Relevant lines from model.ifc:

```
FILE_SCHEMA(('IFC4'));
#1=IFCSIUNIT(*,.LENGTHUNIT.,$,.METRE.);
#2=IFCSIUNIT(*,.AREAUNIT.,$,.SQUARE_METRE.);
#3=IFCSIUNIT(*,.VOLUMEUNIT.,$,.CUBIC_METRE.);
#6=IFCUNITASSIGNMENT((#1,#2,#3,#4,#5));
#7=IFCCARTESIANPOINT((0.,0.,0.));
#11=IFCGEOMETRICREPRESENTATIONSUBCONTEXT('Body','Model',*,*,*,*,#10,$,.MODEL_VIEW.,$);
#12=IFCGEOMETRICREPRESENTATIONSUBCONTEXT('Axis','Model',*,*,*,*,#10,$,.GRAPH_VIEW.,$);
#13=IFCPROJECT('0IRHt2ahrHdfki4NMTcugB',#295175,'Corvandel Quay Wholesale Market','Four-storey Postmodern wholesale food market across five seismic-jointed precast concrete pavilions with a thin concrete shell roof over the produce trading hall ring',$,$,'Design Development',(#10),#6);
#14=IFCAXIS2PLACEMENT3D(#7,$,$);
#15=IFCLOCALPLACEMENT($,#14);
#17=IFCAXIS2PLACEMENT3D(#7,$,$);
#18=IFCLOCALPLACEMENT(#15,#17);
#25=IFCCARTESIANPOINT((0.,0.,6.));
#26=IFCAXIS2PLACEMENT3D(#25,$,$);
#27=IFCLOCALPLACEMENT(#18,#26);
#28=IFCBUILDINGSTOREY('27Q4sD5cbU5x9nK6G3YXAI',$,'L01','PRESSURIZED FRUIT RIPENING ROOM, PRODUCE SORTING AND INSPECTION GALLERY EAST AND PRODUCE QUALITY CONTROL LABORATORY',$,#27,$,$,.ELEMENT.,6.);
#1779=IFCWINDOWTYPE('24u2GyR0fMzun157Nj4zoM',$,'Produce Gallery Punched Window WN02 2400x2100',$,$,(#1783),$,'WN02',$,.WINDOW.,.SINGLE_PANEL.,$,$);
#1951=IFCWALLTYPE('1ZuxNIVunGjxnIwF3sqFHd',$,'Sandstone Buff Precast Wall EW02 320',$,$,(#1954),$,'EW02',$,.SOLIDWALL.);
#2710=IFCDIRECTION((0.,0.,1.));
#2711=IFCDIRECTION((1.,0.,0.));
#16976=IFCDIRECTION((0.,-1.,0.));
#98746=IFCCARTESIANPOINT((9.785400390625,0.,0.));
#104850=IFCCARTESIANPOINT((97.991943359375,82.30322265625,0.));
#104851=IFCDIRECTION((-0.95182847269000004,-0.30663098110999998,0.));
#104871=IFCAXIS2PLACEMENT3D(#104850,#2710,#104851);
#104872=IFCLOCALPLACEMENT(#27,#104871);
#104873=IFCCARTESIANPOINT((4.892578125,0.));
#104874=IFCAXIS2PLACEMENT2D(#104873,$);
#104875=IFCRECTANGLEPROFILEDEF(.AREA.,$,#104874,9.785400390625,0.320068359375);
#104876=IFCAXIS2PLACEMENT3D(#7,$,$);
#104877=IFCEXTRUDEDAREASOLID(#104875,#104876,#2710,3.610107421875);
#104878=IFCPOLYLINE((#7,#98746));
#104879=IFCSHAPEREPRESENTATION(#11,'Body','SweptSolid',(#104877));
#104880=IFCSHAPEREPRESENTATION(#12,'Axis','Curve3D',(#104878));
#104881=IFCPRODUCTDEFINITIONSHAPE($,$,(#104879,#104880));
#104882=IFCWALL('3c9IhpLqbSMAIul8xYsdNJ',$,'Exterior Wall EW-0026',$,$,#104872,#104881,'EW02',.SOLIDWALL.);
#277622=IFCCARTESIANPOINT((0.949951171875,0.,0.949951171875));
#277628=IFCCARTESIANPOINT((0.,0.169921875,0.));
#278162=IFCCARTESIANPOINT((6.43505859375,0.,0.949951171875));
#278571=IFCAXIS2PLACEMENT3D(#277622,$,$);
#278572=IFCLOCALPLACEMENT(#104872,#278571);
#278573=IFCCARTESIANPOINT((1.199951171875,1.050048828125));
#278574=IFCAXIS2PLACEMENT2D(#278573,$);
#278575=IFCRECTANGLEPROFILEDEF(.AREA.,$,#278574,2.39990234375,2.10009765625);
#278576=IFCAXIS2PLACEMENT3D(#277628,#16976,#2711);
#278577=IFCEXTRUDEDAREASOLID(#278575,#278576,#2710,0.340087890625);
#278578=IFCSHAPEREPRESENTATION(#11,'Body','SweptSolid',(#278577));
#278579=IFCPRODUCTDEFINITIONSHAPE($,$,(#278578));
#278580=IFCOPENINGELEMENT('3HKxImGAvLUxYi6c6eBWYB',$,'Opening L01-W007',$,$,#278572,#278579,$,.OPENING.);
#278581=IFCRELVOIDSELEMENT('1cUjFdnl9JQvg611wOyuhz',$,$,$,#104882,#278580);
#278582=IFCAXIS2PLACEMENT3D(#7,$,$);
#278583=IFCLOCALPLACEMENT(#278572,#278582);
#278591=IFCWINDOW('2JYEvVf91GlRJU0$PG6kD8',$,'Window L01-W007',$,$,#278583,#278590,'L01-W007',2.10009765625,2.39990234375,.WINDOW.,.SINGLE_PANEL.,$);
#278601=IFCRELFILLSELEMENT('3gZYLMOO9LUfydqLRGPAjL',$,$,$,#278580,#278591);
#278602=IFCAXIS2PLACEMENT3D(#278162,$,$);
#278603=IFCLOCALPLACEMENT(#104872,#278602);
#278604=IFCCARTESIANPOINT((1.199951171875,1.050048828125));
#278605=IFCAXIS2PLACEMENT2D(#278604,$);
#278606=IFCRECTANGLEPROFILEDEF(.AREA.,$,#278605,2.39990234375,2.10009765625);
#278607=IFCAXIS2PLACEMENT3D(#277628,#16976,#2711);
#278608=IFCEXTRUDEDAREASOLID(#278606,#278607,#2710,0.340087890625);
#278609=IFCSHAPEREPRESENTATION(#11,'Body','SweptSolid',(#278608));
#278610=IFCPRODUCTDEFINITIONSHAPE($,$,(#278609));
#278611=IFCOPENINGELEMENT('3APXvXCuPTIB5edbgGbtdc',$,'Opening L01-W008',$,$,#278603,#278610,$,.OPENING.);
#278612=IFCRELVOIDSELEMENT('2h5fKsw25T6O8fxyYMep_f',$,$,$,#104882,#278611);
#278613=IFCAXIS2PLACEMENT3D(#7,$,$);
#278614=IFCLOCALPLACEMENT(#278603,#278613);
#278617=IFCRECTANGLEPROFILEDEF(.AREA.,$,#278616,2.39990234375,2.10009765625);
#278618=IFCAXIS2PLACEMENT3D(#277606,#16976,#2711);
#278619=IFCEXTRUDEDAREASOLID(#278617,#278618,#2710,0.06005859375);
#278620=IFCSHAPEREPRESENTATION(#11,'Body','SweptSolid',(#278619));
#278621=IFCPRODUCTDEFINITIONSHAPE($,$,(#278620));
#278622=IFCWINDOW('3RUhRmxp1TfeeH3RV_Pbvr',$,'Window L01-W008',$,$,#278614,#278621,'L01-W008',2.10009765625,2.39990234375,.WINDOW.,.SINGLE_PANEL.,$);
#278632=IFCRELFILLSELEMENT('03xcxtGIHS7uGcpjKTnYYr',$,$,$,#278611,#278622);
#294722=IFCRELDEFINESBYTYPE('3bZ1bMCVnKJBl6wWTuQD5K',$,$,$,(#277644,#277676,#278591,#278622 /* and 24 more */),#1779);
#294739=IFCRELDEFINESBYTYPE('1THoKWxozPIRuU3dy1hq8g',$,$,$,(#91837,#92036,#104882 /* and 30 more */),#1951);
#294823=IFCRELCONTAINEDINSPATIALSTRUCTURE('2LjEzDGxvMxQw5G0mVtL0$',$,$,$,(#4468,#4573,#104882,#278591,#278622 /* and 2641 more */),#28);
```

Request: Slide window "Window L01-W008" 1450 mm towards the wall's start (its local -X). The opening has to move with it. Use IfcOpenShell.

```python
import ifcopenshell
import ifcopenshell.api.geometry
import ifcopenshell.util.placement
import ifcopenshell.util.unit

model = ifcopenshell.open("model.ifc")
unit_scale = ifcopenshell.util.unit.calculate_unit_scale(model)

window = model.by_id(278622)
opening = window.FillsVoids[0].RelatingOpeningElement
wall = opening.VoidsElements[0].RelatingBuildingElement

wall_matrix = ifcopenshell.util.placement.get_local_placement(wall.ObjectPlacement)
shift = wall_matrix[:3, 0] * -1.45 / unit_scale
before = ifcopenshell.util.placement.get_local_placement(window.ObjectPlacement)[:3, 3].copy()

# The window is placed relative to its opening, so it follows when the opening moves.
matrix = ifcopenshell.util.placement.get_local_placement(opening.ObjectPlacement)
matrix[:3, 3] += shift
ifcopenshell.api.geometry.edit_object_placement(
    model, product=opening, matrix=matrix, is_si=False, should_transform_children=True
)

after = ifcopenshell.util.placement.get_local_placement(window.ObjectPlacement)[:3, 3]
print("window moved by", (after - before).round(3) + 0.0)

model.write("model-out.ifc")
```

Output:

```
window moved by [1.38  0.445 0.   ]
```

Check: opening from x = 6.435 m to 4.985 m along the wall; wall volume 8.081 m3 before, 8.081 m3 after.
